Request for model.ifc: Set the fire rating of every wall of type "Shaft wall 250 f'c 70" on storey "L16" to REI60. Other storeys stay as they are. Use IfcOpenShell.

First a look at what the model holds.

```python
import ifcopenshell
import ifcopenshell.util.element

model = ifcopenshell.open("model.ifc")
print(model.schema)
storey = next(s for s in model.by_type("IfcBuildingStorey") if s.Name == "L16")
walls = [e for e in ifcopenshell.util.element.get_decomposition(storey) if e.is_a("IfcWall")]
seen = {}
for e in walls:
    element_type = ifcopenshell.util.element.get_type(e)
    key = (element_type.Name if element_type != e and element_type else None, ifcopenshell.util.element.get_pset(e, "Pset_WallCommon", "FireRating"))
    seen[key] = seen.get(key, 0) + 1
for (name, value), count in sorted(seen.items(), key=str):
    print(count, "x", name, "|", value)
```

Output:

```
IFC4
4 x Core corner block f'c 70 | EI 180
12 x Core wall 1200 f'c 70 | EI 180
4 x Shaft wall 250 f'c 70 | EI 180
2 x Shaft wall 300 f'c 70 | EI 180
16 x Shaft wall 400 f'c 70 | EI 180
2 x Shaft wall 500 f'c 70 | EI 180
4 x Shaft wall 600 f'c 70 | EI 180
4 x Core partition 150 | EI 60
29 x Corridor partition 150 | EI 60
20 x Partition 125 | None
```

```python
import ifcopenshell
import ifcopenshell.api.pset
import ifcopenshell.util.element

model = ifcopenshell.open("model.ifc")

storey = next(s for s in model.by_type("IfcBuildingStorey") if s.Name == "L16")
walls = [e for e in ifcopenshell.util.element.get_decomposition(storey) if e.is_a("IfcWall")]

count = 0
for e in walls:
    element_type = ifcopenshell.util.element.get_type(e)
    if element_type in (None, e) or element_type.Name != "Shaft wall 250 f'c 70":
        continue
    # add_pset returns the element's existing set when there is one.
    pset = ifcopenshell.api.pset.add_pset(model, product=e, name="Pset_WallCommon")
    ifcopenshell.api.pset.edit_pset(model, pset=pset, properties={"FireRating": "REI60"})
    count += 1

print(count, "walls updated")

model.write("model_edited.ifc")
```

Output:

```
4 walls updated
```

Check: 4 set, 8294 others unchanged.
